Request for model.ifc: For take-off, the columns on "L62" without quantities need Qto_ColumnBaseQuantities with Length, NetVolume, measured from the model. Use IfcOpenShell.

First a look at what the model holds.

```python
import ifcopenshell
import ifcopenshell.util.element
import ifcopenshell.util.unit

model = ifcopenshell.open("model.ifc")
print(model.schema)
for unit_type in ("LENGTHUNIT", "AREAUNIT", "VOLUMEUNIT"):
    print(unit_type, ifcopenshell.util.unit.calculate_unit_scale(model, unit_type))
storey = next(s for s in model.by_type("IfcBuildingStorey") if s.Name == "L62")
columns = [e for e in ifcopenshell.util.element.get_decomposition(storey) if e.is_a("IfcColumn")]
for e in sorted(columns, key=lambda e: e.id()):
    print(e.id(), e.is_a(), e.Name, list(ifcopenshell.util.element.get_psets(e, qtos_only=True)), sep=" | ")
```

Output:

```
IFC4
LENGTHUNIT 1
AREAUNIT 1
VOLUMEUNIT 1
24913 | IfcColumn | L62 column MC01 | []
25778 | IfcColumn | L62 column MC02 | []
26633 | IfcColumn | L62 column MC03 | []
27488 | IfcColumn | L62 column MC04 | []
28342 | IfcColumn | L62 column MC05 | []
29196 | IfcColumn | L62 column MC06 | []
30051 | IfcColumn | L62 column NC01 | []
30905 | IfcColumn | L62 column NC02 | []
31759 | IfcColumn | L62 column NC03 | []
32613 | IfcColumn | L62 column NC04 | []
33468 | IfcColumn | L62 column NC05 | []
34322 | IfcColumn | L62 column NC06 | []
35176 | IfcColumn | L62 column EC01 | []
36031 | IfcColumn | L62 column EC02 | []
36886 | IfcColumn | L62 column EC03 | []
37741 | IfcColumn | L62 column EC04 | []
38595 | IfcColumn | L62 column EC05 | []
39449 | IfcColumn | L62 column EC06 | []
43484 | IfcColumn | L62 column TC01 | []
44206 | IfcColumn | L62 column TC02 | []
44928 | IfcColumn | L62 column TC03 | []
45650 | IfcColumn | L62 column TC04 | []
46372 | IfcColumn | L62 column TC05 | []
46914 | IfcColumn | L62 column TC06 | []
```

```python
import ifcopenshell
import ifcopenshell.api.pset
import ifcopenshell.geom
import ifcopenshell.util.element
import ifcopenshell.util.shape
import ifcopenshell.util.unit

model = ifcopenshell.open("model.ifc")
unit_scale = ifcopenshell.util.unit.calculate_unit_scale(model)
volume_scale = ifcopenshell.util.unit.calculate_unit_scale(model, "VOLUMEUNIT")
settings = ifcopenshell.geom.settings()

storey = next(s for s in model.by_type("IfcBuildingStorey") if s.Name == "L62")
columns = [e for e in ifcopenshell.util.element.get_decomposition(storey) if e.is_a("IfcColumn")]

for e in sorted(columns, key=lambda e: e.id()):
    if ifcopenshell.util.element.get_psets(e, qtos_only=True, should_inherit=False):
        continue
    # Geometry comes back in metres, in the element's own axes.
    shape = ifcopenshell.geom.create_shape(settings, e)
    values = {
        "Length": ifcopenshell.util.shape.get_z(shape.geometry) / unit_scale,
        "NetVolume": ifcopenshell.util.shape.get_volume(shape.geometry) / volume_scale,
    }
    qto = ifcopenshell.api.pset.add_qto(model, product=e, name="Qto_ColumnBaseQuantities")
    ifcopenshell.api.pset.edit_qto(model, qto=qto, properties=values)
    print(e.id(), {k: round(v, 3) for k, v in values.items()})

model.write("model-out.ifc")
```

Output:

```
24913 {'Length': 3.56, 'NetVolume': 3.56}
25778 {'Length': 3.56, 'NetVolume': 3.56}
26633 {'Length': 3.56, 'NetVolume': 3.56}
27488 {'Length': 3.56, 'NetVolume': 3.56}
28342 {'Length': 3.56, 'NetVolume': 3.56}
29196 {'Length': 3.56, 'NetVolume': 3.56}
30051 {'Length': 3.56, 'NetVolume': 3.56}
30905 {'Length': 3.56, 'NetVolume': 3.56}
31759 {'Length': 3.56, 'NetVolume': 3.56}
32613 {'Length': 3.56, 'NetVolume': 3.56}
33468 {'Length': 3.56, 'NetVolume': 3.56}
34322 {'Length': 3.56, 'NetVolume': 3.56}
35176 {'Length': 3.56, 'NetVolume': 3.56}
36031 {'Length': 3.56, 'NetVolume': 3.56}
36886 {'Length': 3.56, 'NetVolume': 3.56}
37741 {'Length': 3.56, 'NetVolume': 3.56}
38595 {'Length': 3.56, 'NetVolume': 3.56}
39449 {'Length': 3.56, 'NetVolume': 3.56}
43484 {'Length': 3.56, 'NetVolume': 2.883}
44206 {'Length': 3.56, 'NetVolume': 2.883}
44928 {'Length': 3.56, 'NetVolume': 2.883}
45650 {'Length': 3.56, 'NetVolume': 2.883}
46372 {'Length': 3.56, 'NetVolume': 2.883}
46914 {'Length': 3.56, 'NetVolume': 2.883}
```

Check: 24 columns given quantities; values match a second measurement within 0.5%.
